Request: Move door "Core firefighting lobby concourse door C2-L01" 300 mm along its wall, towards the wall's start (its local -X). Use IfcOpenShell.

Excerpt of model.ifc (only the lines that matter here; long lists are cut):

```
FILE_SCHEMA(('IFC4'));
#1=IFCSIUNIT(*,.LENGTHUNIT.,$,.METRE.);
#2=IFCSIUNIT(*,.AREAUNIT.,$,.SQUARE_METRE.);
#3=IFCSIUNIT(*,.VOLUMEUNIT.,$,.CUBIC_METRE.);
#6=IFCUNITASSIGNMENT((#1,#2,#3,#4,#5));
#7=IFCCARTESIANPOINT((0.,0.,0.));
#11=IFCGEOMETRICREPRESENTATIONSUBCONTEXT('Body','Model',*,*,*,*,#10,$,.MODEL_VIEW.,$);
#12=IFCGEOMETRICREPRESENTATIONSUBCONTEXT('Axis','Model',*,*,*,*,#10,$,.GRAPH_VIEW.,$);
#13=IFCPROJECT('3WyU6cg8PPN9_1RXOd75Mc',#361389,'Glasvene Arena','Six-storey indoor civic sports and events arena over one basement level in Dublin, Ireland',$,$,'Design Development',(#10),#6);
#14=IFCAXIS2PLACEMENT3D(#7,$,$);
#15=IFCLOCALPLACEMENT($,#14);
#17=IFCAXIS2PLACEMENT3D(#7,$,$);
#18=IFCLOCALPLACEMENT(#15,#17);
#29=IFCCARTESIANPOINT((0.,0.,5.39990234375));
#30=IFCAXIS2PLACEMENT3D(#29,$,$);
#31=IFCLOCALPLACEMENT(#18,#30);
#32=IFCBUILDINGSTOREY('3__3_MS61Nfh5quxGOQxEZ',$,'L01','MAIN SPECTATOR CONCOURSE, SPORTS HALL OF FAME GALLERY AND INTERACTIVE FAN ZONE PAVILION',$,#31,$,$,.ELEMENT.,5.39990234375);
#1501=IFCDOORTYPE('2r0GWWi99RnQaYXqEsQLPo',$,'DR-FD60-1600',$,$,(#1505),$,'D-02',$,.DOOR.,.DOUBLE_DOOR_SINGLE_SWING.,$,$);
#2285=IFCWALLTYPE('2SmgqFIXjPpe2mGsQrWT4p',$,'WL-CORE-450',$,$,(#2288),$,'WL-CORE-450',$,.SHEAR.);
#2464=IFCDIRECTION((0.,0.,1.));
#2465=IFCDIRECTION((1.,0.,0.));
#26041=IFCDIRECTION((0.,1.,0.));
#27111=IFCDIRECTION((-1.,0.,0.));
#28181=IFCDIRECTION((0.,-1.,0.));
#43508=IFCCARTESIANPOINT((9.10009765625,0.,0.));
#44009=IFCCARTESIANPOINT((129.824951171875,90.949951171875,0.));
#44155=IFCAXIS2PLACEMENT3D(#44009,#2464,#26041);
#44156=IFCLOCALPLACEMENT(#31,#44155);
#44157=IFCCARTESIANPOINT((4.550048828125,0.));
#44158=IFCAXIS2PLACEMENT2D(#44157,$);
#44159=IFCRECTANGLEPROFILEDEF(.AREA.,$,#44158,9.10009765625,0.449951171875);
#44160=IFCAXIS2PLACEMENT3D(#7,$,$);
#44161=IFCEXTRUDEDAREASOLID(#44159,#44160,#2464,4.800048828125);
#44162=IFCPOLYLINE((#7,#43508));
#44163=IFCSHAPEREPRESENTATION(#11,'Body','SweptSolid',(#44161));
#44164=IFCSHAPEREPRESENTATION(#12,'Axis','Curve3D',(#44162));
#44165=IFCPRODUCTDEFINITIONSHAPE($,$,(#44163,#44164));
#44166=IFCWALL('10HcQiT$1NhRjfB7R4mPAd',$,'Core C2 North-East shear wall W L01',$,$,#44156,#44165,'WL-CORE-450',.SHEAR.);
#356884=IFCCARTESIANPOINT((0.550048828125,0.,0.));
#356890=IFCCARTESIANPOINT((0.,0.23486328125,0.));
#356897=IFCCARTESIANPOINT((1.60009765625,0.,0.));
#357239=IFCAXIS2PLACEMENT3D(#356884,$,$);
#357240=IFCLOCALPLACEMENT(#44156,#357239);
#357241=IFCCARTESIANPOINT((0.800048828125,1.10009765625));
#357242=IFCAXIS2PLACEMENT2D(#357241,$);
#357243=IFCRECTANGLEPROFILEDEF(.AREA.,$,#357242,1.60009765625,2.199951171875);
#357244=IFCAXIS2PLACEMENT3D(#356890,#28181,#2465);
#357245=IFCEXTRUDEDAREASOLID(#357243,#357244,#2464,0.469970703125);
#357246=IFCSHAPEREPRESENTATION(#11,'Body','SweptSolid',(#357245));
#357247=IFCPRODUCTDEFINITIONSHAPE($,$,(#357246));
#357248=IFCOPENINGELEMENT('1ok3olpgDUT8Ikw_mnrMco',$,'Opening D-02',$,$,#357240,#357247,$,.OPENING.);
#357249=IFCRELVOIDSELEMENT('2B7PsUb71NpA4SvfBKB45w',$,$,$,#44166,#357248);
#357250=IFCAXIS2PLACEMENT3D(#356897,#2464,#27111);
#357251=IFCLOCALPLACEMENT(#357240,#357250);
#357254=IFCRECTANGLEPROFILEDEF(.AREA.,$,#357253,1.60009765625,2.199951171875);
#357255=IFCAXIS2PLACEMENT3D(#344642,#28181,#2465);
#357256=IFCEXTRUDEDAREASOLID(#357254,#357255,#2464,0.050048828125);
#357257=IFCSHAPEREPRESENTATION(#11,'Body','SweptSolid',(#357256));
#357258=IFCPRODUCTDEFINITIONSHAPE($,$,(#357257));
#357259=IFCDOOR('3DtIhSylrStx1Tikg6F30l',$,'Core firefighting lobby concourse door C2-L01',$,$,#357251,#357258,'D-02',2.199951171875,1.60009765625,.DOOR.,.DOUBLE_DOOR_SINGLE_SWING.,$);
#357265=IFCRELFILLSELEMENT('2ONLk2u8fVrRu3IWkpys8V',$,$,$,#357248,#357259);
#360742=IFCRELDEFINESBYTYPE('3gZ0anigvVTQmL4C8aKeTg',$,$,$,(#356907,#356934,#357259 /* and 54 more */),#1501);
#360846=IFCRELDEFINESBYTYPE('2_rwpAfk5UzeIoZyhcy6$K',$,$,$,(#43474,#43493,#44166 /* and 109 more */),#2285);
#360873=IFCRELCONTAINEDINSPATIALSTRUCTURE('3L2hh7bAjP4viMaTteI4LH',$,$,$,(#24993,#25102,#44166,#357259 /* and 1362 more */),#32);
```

```python
import ifcopenshell
import ifcopenshell.api.geometry
import ifcopenshell.util.placement
import ifcopenshell.util.unit

model = ifcopenshell.open("model.ifc")
unit_scale = ifcopenshell.util.unit.calculate_unit_scale(model)

door = model.by_guid("3DtIhSylrStx1Tikg6F30l")
opening = door.FillsVoids[0].RelatingOpeningElement
wall = opening.VoidsElements[0].RelatingBuildingElement

wall_matrix = ifcopenshell.util.placement.get_local_placement(wall.ObjectPlacement)
shift = wall_matrix[:3, 0] * -0.3 / unit_scale
before = ifcopenshell.util.placement.get_local_placement(door.ObjectPlacement)[:3, 3].copy()

# The door is placed relative to its opening, so it follows when the opening moves.
matrix = ifcopenshell.util.placement.get_local_placement(opening.ObjectPlacement)
matrix[:3, 3] += shift
ifcopenshell.api.geometry.edit_object_placement(
    model, product=opening, matrix=matrix, is_si=False, should_transform_children=True
)

after = ifcopenshell.util.placement.get_local_placement(door.ObjectPlacement)[:3, 3]
print("door moved by", (after - before).round(3) + 0.0)

model.write("model_rev.ifc")
```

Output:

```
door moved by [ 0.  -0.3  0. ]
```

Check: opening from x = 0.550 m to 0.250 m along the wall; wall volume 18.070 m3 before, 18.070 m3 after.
